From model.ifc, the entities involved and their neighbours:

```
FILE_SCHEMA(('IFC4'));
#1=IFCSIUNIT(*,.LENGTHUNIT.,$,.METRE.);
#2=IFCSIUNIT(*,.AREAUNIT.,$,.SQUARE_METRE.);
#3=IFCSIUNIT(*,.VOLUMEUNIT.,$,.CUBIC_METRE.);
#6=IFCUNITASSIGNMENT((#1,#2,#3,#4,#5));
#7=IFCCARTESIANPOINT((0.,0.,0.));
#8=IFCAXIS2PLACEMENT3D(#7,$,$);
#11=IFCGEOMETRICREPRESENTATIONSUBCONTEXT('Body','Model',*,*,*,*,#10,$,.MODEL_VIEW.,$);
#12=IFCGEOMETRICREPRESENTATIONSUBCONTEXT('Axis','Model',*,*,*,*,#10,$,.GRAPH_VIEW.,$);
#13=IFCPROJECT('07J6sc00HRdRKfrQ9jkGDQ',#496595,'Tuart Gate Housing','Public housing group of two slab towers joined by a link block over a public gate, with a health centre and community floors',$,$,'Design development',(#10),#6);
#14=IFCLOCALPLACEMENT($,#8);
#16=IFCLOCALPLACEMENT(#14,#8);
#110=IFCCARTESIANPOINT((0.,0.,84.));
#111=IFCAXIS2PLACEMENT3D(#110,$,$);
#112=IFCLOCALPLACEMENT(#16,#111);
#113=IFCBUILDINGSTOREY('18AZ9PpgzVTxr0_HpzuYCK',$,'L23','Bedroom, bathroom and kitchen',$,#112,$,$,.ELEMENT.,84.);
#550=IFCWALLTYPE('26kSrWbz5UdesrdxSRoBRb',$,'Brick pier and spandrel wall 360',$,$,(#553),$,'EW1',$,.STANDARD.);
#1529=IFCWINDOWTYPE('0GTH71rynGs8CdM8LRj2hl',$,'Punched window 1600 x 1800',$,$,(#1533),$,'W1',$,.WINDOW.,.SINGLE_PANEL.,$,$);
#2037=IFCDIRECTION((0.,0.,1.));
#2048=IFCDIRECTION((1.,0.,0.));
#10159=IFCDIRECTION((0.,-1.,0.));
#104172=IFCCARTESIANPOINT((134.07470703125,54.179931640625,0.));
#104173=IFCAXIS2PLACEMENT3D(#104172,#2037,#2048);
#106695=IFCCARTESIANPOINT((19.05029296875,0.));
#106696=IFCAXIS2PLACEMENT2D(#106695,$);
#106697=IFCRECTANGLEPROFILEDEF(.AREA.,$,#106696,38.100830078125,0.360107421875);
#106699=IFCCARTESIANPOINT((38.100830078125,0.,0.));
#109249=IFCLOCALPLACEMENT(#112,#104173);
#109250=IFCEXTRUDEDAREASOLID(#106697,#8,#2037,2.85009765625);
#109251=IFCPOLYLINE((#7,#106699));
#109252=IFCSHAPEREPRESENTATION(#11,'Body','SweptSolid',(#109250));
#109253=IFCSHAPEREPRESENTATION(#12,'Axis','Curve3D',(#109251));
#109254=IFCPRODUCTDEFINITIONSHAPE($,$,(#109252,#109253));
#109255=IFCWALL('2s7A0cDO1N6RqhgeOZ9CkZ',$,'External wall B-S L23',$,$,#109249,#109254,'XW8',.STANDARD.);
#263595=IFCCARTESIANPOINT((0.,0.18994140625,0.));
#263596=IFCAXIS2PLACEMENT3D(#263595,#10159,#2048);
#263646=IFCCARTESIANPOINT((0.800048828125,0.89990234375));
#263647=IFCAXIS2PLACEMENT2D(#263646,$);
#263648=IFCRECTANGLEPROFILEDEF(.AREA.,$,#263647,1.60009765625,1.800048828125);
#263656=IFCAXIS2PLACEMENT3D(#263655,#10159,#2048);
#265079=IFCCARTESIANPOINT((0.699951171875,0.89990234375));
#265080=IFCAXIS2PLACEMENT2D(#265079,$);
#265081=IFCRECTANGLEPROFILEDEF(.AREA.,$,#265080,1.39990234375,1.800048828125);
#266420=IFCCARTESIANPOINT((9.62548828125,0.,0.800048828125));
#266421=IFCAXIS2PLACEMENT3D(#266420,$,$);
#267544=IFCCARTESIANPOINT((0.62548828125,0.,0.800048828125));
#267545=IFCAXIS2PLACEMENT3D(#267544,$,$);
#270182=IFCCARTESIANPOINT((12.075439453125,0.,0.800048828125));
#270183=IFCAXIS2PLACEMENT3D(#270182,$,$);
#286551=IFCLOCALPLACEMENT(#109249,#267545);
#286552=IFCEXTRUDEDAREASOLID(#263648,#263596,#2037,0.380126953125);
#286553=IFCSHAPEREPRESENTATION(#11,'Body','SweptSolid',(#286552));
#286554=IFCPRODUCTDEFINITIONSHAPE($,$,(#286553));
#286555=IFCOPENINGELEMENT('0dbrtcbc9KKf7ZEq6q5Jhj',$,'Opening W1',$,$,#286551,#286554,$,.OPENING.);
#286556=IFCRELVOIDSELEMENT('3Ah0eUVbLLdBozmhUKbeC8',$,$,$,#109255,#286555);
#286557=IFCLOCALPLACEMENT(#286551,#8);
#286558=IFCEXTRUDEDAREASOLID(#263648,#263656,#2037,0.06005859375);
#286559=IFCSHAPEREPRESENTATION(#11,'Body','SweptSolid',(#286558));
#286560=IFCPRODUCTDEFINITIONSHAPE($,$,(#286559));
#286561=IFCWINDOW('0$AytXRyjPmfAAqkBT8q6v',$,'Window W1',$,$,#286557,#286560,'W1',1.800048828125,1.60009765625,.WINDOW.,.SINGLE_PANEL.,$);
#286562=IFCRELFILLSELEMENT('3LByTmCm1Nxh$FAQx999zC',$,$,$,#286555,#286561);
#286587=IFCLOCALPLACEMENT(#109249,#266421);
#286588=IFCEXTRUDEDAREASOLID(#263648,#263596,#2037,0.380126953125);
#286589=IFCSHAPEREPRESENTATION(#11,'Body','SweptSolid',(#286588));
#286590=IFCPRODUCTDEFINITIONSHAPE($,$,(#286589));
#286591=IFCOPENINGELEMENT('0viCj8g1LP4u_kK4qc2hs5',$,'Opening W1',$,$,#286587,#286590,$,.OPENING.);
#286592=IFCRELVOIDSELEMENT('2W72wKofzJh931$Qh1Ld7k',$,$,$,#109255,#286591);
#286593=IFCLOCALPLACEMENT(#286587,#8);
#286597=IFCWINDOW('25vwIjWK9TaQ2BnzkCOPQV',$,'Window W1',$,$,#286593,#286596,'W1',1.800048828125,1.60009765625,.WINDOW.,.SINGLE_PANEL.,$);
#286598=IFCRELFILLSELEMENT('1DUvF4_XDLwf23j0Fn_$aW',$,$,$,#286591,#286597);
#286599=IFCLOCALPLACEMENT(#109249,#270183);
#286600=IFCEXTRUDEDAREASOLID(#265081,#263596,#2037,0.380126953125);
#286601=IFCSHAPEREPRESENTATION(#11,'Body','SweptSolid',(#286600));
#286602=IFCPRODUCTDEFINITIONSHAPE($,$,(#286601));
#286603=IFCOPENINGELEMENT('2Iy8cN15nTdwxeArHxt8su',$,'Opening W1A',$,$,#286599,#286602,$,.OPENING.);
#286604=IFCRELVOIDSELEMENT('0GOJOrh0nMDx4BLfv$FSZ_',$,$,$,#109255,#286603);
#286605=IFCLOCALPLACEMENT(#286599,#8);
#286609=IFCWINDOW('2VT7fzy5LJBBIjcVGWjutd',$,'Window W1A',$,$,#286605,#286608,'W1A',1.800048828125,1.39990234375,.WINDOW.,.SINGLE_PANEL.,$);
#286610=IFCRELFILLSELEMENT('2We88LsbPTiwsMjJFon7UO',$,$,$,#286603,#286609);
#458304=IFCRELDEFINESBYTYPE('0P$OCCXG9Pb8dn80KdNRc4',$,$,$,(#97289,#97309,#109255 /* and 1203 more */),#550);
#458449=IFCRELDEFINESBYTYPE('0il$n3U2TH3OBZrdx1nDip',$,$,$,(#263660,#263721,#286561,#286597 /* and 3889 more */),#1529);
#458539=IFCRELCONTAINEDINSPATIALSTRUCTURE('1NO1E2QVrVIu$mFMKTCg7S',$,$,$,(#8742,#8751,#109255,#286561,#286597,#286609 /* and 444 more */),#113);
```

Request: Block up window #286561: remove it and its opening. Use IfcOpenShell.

```python
import ifcopenshell
import ifcopenshell.api.feature
import ifcopenshell.api.root
import ifcopenshell.geom
import ifcopenshell.util.shape

model = ifcopenshell.open("model.ifc")
settings = ifcopenshell.geom.settings()


def volume(element):
    """Net volume in cubic metres, openings subtracted."""
    shape = ifcopenshell.geom.create_shape(settings, element)
    return ifcopenshell.util.shape.get_volume(shape.geometry)


window = model.by_id(286561)
opening = window.FillsVoids[0].RelatingOpeningElement
wall = opening.VoidsElements[0].RelatingBuildingElement
before = volume(wall)

ifcopenshell.api.root.remove_product(model, product=window)
ifcopenshell.api.feature.remove_feature(model, feature=opening)

after = volume(wall)

print(f"wall volume {before:.3f} -> {after:.3f} m3")

model.write("model_edited.ifc")
```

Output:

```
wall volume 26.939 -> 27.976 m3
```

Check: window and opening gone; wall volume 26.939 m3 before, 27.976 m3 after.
